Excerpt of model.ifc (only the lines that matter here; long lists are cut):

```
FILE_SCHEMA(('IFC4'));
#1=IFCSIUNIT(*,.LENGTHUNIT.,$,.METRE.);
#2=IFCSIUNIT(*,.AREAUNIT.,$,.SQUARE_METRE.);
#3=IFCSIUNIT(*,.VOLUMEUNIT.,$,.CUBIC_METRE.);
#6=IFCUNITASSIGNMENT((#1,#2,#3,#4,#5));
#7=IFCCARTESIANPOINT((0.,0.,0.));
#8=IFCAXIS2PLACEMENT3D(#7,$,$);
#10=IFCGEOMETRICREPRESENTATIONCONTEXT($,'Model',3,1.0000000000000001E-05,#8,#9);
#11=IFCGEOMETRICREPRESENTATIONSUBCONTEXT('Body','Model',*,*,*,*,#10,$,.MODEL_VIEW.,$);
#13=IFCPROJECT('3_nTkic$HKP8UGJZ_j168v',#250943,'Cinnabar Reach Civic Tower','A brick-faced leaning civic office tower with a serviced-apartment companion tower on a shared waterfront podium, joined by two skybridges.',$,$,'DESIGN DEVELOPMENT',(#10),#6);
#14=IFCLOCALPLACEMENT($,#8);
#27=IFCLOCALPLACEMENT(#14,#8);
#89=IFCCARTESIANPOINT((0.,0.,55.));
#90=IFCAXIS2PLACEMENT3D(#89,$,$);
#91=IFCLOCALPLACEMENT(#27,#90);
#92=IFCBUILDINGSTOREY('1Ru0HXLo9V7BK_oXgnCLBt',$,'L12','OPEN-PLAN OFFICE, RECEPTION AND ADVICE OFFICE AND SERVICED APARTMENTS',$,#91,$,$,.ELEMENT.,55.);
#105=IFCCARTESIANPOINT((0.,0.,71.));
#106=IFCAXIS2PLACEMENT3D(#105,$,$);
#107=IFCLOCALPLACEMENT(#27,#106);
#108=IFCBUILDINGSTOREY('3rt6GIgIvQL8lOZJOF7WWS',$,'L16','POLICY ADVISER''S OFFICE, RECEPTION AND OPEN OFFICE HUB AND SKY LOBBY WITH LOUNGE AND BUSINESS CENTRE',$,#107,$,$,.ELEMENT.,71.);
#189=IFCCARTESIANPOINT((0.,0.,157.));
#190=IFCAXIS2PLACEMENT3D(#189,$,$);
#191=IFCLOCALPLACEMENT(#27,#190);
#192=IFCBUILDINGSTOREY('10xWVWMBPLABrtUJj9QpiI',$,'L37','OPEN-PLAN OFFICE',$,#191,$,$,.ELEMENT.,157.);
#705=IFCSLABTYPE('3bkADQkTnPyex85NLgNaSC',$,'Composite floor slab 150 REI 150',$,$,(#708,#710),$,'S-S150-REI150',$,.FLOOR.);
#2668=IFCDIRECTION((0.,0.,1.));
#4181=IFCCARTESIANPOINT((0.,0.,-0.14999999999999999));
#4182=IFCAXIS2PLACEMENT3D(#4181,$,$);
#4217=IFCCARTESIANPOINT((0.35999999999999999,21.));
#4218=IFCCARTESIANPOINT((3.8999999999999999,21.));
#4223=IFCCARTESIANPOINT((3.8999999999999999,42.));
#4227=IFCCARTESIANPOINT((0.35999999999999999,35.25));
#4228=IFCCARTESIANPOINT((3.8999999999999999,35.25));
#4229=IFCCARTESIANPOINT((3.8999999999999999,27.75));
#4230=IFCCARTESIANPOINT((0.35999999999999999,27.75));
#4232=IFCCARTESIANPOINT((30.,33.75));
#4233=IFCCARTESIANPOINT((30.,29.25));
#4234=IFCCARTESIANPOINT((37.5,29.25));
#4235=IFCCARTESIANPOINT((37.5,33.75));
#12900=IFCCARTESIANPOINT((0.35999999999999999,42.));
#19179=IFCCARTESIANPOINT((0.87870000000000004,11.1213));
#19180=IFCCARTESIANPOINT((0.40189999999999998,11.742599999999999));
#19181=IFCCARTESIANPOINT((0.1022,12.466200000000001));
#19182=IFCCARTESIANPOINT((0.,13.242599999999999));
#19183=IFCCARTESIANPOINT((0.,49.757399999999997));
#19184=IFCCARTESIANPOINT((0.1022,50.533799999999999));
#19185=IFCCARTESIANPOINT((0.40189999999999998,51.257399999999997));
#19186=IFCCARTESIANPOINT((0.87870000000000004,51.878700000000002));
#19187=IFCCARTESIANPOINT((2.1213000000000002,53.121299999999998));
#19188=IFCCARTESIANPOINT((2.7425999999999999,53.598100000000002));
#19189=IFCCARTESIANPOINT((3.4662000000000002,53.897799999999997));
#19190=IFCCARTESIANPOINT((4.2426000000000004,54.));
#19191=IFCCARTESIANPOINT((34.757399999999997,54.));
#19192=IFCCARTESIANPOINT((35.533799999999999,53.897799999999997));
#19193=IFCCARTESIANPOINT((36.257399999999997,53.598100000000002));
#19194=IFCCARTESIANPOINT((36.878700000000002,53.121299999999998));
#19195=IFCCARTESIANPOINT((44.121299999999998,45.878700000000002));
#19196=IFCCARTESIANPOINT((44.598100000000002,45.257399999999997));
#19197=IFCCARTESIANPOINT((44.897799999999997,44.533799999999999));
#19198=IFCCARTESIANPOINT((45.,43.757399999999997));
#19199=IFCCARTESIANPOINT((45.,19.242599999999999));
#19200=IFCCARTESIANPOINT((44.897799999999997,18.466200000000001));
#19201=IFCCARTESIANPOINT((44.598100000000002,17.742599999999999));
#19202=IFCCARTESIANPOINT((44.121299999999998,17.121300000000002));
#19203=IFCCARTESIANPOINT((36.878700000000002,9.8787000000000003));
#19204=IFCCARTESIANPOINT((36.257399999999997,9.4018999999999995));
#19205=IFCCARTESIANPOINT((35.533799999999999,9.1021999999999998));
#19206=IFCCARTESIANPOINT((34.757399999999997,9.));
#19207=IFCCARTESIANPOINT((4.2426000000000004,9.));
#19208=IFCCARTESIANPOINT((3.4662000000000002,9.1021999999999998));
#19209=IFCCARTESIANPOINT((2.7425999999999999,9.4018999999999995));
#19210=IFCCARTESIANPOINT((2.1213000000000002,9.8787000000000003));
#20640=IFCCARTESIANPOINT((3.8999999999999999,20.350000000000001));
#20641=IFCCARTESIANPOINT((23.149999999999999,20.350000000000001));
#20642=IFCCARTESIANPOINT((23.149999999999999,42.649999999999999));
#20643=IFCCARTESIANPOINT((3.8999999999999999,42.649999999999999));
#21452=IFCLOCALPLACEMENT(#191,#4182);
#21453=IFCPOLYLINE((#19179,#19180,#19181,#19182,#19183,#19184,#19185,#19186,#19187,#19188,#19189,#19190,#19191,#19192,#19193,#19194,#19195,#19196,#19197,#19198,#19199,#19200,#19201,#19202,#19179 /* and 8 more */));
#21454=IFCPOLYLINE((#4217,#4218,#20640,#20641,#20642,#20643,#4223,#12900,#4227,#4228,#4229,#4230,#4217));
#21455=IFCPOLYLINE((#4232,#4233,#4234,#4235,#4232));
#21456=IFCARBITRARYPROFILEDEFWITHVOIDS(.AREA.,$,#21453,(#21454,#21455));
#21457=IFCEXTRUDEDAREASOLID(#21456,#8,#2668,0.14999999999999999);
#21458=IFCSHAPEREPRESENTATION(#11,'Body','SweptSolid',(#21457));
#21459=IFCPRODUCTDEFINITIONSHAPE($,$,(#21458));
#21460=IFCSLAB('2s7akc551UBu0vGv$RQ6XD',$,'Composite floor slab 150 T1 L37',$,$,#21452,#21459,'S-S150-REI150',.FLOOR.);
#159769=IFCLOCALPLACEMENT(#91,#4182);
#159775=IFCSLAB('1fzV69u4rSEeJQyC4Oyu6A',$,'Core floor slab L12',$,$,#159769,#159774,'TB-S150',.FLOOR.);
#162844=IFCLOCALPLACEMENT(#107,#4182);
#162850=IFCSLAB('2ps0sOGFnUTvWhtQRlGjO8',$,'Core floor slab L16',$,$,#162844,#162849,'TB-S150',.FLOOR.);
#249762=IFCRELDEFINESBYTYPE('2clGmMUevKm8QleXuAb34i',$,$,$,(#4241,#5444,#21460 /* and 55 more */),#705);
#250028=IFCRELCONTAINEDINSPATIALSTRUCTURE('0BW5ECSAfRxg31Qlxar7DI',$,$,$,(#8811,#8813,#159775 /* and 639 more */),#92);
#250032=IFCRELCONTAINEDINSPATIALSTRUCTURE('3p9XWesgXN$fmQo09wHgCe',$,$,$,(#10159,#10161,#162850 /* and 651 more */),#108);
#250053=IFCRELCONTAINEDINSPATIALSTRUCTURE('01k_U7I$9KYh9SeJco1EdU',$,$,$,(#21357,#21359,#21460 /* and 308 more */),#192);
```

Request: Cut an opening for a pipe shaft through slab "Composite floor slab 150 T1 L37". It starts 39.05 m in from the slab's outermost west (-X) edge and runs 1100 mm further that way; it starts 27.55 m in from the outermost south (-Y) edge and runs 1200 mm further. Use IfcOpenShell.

```python
import numpy as np
import ifcopenshell
import ifcopenshell.api.feature
import ifcopenshell.api.geometry
import ifcopenshell.api.root
import ifcopenshell.geom
import ifcopenshell.util.placement
import ifcopenshell.util.representation
import ifcopenshell.util.shape
import ifcopenshell.util.unit

model = ifcopenshell.open("model.ifc")
unit_scale = ifcopenshell.util.unit.calculate_unit_scale(model)
settings = ifcopenshell.geom.settings()


def volume(element):
    """Net volume in cubic metres, openings subtracted."""
    shape = ifcopenshell.geom.create_shape(settings, element)
    return ifcopenshell.util.shape.get_volume(shape.geometry)


slab = model.by_guid("2s7akc551UBu0vGv$RQ6XD")
before = volume(slab)

# Extent in the slab's own axes, in metres. The edges named are its -X and -Y sides.
slab_shape = ifcopenshell.geom.create_shape(settings, slab)
vertices = ifcopenshell.util.shape.get_vertices(slab_shape.geometry)
x_min, y_min, bottom = vertices.min(axis=0)
top = vertices[:, 2].max()

opening = ifcopenshell.api.root.create_entity(model, ifc_class="IfcOpeningElement", name="Pipe shaft opening", predefined_type="OPENING")
context = ifcopenshell.util.representation.get_context(model, "Model", "Body", "MODEL_VIEW")
width, depth = 1.1, 1.2
outline = [(0.0, 0.0), (width, 0.0), (width, depth), (0.0, depth), (0.0, 0.0)]
# Overshoot both faces by 50 mm so the cut is clean.
shape = ifcopenshell.api.geometry.add_slab_representation(
    model, context=context, depth=top - bottom + 0.1, polyline=outline
)
ifcopenshell.api.geometry.assign_representation(model, product=opening, representation=shape)

matrix = ifcopenshell.util.placement.get_local_placement(slab.ObjectPlacement)
matrix[:, 3] = matrix @ np.append(np.array([x_min + 39.05, y_min + 27.55, bottom - 0.05]) / unit_scale, 1.0)
ifcopenshell.api.geometry.edit_object_placement(model, product=opening, matrix=matrix, is_si=False)
ifcopenshell.api.feature.add_feature(model, feature=opening, element=slab)

after = volume(slab)

print(f"slab volume {before:.3f} -> {after:.3f} m3")

model.write("model_v2.ifc")
```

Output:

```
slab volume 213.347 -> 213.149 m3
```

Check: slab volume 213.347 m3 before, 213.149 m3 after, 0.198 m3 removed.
